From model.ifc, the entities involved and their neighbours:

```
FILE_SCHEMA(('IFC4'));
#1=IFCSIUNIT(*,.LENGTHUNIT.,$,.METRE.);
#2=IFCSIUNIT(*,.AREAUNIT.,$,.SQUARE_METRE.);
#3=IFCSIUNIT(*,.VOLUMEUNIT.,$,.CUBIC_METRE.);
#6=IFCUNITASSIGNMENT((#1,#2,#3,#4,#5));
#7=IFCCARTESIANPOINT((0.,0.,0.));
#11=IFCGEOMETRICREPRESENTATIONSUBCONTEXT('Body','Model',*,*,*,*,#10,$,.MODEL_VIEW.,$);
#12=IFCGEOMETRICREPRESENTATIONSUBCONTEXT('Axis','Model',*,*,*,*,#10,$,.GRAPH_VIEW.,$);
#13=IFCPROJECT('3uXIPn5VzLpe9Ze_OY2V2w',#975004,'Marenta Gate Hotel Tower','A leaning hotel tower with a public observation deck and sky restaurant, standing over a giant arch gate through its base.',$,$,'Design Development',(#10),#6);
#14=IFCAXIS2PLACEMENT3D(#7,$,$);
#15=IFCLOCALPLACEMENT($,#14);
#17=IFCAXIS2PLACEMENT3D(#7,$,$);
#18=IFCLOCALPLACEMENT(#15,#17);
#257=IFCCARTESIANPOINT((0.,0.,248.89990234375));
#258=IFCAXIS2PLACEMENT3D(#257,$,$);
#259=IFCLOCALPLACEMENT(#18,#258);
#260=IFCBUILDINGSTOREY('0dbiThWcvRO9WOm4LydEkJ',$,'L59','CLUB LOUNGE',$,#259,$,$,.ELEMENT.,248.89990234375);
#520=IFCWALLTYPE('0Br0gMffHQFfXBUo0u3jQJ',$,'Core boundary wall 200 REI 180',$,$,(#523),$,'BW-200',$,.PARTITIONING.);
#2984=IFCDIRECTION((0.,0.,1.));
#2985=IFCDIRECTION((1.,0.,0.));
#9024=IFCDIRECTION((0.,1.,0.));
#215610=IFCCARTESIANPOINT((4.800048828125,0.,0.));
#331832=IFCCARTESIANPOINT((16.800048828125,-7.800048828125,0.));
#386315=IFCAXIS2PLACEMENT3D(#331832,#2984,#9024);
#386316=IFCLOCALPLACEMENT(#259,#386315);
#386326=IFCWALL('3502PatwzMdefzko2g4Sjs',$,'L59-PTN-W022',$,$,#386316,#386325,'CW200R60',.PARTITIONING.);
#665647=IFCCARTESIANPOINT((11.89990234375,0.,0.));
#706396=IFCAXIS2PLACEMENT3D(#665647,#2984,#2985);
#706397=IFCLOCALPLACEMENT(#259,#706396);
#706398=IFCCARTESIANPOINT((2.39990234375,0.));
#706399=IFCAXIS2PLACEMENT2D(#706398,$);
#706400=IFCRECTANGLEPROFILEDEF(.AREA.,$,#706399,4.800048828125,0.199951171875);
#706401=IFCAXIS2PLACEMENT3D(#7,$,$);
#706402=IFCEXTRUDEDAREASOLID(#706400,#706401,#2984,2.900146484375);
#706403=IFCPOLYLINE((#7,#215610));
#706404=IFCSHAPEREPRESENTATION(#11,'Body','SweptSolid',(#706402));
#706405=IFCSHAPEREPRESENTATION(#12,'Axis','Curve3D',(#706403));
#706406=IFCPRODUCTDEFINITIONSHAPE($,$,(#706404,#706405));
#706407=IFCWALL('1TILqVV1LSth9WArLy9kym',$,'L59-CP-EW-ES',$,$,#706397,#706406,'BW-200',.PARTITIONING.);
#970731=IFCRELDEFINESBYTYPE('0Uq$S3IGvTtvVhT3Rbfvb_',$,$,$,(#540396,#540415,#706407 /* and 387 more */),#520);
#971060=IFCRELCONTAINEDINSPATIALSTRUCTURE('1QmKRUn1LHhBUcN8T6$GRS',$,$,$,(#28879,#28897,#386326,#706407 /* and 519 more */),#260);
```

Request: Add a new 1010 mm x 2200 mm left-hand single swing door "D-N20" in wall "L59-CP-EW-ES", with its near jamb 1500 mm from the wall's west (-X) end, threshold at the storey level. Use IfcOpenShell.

```python
import numpy as np
import ifcopenshell
import ifcopenshell.api.feature
import ifcopenshell.api.geometry
import ifcopenshell.api.root
import ifcopenshell.api.spatial
import ifcopenshell.geom
import ifcopenshell.util.element
import ifcopenshell.util.placement
import ifcopenshell.util.representation
import ifcopenshell.util.shape
import ifcopenshell.util.unit

model = ifcopenshell.open("model.ifc")
unit_scale = ifcopenshell.util.unit.calculate_unit_scale(model)
settings = ifcopenshell.geom.settings()


def volume(element):
    """Net volume in cubic metres, openings subtracted."""
    shape = ifcopenshell.geom.create_shape(settings, element)
    return ifcopenshell.util.shape.get_volume(shape.geometry)


wall = model.by_guid("1TILqVV1LSth9WArLy9kym")
storey = ifcopenshell.util.element.get_container(wall, ifc_class="IfcBuildingStorey")
context = ifcopenshell.util.representation.get_context(model, "Model", "Body", "MODEL_VIEW")
before = volume(wall)

width, height, from_end, sill = 1.01, 2.2, 1.5, 0.0  # metres

# The wall runs along its own X axis, and the end named is its -X end.
wall_shape = ifcopenshell.geom.create_shape(settings, wall)
x, y, z = ifcopenshell.util.shape.get_vertices(wall_shape.geometry).T
start = x.min() + from_end
face, thickness = float(y.min()), float(y.max() - y.min())
wall_matrix = ifcopenshell.util.placement.get_local_placement(wall.ObjectPlacement)
level = ifcopenshell.util.placement.get_local_placement(storey.ObjectPlacement)[2, 3]


def in_wall(x, y):
    """Placement at x, y metres in the wall's axes, at sill height."""
    matrix = wall_matrix.copy()
    matrix[:, 3] = wall_matrix @ np.array([x / unit_scale, y / unit_scale, 0.0, 1.0])
    matrix[2, 3] = level + sill / unit_scale
    return matrix


# Opening: a box that overshoots both wall faces by 50 mm.
opening = ifcopenshell.api.root.create_entity(model, ifc_class="IfcOpeningElement", predefined_type="OPENING")
box = ifcopenshell.api.geometry.add_wall_representation(
    model, context=context, length=width, height=height, thickness=thickness + 0.1
)
ifcopenshell.api.geometry.assign_representation(model, product=opening, representation=box)
ifcopenshell.api.geometry.edit_object_placement(model, product=opening, matrix=in_wall(start, face - 0.05), is_si=False)
ifcopenshell.api.feature.add_feature(model, feature=opening, element=wall)

door = ifcopenshell.api.root.create_entity(model, ifc_class="IfcDoor", name="D-N20", predefined_type="DOOR")
door.OverallWidth, door.OverallHeight = width / unit_scale, height / unit_scale
door.OperationType = "SINGLE_SWING_LEFT"
body = ifcopenshell.api.geometry.add_door_representation(
    model,
    context=context,
    overall_width=door.OverallWidth,
    overall_height=door.OverallHeight,
    operation_type="SINGLE_SWING_LEFT",
    lining_properties={"LiningDepth": thickness / unit_scale, "ThresholdDepth": thickness / unit_scale},
)
ifcopenshell.api.geometry.assign_representation(model, product=door, representation=body)
ifcopenshell.api.spatial.assign_container(model, products=[door], relating_structure=storey)
ifcopenshell.api.feature.add_filling(model, opening=opening, element=door)

# The lining spans the wall, so the door starts at the wall face.
ifcopenshell.api.geometry.edit_object_placement(model, product=door, matrix=in_wall(start, face), is_si=False)

after = volume(wall)

print(f"wall volume {before:.3f} -> {after:.3f} m3")

model.write("model_v2.ifc")
```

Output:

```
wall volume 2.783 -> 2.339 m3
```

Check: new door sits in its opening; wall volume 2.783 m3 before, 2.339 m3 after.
